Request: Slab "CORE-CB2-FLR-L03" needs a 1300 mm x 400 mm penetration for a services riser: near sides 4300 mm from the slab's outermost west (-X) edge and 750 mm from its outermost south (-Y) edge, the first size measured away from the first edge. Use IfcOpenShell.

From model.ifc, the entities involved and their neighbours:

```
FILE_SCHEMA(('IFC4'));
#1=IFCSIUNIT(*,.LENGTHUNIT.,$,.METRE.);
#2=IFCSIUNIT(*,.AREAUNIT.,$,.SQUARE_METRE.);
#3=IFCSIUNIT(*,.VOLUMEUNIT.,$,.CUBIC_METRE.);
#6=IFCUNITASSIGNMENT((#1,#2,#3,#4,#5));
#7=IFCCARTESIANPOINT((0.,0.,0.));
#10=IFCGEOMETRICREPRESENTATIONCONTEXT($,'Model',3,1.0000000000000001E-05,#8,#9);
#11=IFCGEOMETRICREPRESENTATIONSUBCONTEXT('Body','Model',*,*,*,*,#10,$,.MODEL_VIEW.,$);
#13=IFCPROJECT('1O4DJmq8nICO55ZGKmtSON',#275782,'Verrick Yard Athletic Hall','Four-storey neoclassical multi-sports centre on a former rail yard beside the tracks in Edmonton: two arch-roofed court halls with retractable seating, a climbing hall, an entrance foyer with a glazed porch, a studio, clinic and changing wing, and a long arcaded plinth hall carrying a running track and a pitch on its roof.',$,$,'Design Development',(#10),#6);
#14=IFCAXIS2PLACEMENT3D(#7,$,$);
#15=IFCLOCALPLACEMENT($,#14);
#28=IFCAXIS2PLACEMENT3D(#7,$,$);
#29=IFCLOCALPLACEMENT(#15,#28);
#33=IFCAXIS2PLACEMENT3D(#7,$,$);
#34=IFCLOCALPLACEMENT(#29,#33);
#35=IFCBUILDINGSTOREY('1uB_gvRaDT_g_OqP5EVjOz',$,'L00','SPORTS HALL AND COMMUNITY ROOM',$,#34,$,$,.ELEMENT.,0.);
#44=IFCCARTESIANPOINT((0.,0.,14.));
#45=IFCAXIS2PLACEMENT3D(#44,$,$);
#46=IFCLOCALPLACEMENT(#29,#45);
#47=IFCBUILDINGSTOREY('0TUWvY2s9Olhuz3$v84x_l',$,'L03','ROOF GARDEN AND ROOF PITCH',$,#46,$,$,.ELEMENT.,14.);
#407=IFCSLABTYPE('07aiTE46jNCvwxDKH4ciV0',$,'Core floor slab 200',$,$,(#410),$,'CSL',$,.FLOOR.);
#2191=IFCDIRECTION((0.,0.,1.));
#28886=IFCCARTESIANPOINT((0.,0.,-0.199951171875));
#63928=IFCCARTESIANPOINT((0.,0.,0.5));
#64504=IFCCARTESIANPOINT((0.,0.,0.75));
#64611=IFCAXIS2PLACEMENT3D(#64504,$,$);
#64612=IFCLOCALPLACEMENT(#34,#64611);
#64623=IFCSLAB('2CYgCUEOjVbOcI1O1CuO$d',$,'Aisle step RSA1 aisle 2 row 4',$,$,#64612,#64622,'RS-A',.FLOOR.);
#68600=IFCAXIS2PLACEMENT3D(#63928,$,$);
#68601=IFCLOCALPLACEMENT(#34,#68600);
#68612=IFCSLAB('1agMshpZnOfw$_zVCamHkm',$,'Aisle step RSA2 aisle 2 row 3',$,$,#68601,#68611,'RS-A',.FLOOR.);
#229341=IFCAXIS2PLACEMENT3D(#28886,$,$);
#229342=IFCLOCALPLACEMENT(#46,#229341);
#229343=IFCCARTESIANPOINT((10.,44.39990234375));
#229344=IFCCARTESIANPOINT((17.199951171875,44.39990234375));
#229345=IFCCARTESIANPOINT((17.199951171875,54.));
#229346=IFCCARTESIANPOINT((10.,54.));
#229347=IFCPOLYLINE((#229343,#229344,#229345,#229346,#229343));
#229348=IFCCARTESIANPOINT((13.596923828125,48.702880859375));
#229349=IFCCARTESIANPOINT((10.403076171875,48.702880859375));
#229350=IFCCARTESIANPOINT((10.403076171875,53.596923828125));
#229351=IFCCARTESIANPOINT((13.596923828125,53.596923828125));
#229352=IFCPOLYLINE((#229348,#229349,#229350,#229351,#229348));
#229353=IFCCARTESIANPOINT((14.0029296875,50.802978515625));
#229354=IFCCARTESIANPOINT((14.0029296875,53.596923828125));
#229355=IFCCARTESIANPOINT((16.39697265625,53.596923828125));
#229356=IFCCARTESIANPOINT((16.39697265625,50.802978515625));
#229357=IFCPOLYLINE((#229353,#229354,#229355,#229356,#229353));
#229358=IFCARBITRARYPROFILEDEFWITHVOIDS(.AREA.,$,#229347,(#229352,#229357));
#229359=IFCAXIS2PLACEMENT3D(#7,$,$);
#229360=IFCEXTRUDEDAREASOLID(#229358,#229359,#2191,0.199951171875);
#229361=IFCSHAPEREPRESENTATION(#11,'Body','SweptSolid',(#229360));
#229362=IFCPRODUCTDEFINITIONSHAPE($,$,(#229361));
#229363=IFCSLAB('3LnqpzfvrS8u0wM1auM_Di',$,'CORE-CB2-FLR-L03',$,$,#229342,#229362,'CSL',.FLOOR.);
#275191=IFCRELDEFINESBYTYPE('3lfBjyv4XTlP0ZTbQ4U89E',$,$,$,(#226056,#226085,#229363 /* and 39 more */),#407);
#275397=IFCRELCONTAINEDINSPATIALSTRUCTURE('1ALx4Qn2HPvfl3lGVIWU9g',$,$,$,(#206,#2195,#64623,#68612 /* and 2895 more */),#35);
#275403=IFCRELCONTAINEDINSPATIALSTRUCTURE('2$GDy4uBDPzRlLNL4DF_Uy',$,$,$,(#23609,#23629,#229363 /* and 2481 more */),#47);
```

```python
import numpy as np
import ifcopenshell
import ifcopenshell.api.feature
import ifcopenshell.api.geometry
import ifcopenshell.api.root
import ifcopenshell.geom
import ifcopenshell.util.placement
import ifcopenshell.util.representation
import ifcopenshell.util.shape
import ifcopenshell.util.unit

model = ifcopenshell.open("model.ifc")
unit_scale = ifcopenshell.util.unit.calculate_unit_scale(model)
settings = ifcopenshell.geom.settings()


def volume(element):
    """Net volume in cubic metres, openings subtracted."""
    shape = ifcopenshell.geom.create_shape(settings, element)
    return ifcopenshell.util.shape.get_volume(shape.geometry)


slab = model.by_guid("3LnqpzfvrS8u0wM1auM_Di")
before = volume(slab)

# Extent in the slab's own axes, in metres. The edges named are its -X and -Y sides.
slab_shape = ifcopenshell.geom.create_shape(settings, slab)
vertices = ifcopenshell.util.shape.get_vertices(slab_shape.geometry)
x_min, y_min, bottom = vertices.min(axis=0)
top = vertices[:, 2].max()

opening = ifcopenshell.api.root.create_entity(model, ifc_class="IfcOpeningElement", name="Services riser opening", predefined_type="OPENING")
context = ifcopenshell.util.representation.get_context(model, "Model", "Body", "MODEL_VIEW")
width, depth = 1.3, 0.4
outline = [(0.0, 0.0), (width, 0.0), (width, depth), (0.0, depth), (0.0, 0.0)]
# Overshoot both faces by 50 mm so the cut is clean.
shape = ifcopenshell.api.geometry.add_slab_representation(
    model, context=context, depth=top - bottom + 0.1, polyline=outline
)
ifcopenshell.api.geometry.assign_representation(model, product=opening, representation=shape)

matrix = ifcopenshell.util.placement.get_local_placement(slab.ObjectPlacement)
matrix[:, 3] = matrix @ np.append(np.array([x_min + 4.3, y_min + 0.75, bottom - 0.05]) / unit_scale, 1.0)
ifcopenshell.api.geometry.edit_object_placement(model, product=opening, matrix=matrix, is_si=False)
ifcopenshell.api.feature.add_feature(model, feature=opening, element=slab)

after = volume(slab)

print(f"slab volume {before:.3f} -> {after:.3f} m3")

model.write("model_edited.ifc")
```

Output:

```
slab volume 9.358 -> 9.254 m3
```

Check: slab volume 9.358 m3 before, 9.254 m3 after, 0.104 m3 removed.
